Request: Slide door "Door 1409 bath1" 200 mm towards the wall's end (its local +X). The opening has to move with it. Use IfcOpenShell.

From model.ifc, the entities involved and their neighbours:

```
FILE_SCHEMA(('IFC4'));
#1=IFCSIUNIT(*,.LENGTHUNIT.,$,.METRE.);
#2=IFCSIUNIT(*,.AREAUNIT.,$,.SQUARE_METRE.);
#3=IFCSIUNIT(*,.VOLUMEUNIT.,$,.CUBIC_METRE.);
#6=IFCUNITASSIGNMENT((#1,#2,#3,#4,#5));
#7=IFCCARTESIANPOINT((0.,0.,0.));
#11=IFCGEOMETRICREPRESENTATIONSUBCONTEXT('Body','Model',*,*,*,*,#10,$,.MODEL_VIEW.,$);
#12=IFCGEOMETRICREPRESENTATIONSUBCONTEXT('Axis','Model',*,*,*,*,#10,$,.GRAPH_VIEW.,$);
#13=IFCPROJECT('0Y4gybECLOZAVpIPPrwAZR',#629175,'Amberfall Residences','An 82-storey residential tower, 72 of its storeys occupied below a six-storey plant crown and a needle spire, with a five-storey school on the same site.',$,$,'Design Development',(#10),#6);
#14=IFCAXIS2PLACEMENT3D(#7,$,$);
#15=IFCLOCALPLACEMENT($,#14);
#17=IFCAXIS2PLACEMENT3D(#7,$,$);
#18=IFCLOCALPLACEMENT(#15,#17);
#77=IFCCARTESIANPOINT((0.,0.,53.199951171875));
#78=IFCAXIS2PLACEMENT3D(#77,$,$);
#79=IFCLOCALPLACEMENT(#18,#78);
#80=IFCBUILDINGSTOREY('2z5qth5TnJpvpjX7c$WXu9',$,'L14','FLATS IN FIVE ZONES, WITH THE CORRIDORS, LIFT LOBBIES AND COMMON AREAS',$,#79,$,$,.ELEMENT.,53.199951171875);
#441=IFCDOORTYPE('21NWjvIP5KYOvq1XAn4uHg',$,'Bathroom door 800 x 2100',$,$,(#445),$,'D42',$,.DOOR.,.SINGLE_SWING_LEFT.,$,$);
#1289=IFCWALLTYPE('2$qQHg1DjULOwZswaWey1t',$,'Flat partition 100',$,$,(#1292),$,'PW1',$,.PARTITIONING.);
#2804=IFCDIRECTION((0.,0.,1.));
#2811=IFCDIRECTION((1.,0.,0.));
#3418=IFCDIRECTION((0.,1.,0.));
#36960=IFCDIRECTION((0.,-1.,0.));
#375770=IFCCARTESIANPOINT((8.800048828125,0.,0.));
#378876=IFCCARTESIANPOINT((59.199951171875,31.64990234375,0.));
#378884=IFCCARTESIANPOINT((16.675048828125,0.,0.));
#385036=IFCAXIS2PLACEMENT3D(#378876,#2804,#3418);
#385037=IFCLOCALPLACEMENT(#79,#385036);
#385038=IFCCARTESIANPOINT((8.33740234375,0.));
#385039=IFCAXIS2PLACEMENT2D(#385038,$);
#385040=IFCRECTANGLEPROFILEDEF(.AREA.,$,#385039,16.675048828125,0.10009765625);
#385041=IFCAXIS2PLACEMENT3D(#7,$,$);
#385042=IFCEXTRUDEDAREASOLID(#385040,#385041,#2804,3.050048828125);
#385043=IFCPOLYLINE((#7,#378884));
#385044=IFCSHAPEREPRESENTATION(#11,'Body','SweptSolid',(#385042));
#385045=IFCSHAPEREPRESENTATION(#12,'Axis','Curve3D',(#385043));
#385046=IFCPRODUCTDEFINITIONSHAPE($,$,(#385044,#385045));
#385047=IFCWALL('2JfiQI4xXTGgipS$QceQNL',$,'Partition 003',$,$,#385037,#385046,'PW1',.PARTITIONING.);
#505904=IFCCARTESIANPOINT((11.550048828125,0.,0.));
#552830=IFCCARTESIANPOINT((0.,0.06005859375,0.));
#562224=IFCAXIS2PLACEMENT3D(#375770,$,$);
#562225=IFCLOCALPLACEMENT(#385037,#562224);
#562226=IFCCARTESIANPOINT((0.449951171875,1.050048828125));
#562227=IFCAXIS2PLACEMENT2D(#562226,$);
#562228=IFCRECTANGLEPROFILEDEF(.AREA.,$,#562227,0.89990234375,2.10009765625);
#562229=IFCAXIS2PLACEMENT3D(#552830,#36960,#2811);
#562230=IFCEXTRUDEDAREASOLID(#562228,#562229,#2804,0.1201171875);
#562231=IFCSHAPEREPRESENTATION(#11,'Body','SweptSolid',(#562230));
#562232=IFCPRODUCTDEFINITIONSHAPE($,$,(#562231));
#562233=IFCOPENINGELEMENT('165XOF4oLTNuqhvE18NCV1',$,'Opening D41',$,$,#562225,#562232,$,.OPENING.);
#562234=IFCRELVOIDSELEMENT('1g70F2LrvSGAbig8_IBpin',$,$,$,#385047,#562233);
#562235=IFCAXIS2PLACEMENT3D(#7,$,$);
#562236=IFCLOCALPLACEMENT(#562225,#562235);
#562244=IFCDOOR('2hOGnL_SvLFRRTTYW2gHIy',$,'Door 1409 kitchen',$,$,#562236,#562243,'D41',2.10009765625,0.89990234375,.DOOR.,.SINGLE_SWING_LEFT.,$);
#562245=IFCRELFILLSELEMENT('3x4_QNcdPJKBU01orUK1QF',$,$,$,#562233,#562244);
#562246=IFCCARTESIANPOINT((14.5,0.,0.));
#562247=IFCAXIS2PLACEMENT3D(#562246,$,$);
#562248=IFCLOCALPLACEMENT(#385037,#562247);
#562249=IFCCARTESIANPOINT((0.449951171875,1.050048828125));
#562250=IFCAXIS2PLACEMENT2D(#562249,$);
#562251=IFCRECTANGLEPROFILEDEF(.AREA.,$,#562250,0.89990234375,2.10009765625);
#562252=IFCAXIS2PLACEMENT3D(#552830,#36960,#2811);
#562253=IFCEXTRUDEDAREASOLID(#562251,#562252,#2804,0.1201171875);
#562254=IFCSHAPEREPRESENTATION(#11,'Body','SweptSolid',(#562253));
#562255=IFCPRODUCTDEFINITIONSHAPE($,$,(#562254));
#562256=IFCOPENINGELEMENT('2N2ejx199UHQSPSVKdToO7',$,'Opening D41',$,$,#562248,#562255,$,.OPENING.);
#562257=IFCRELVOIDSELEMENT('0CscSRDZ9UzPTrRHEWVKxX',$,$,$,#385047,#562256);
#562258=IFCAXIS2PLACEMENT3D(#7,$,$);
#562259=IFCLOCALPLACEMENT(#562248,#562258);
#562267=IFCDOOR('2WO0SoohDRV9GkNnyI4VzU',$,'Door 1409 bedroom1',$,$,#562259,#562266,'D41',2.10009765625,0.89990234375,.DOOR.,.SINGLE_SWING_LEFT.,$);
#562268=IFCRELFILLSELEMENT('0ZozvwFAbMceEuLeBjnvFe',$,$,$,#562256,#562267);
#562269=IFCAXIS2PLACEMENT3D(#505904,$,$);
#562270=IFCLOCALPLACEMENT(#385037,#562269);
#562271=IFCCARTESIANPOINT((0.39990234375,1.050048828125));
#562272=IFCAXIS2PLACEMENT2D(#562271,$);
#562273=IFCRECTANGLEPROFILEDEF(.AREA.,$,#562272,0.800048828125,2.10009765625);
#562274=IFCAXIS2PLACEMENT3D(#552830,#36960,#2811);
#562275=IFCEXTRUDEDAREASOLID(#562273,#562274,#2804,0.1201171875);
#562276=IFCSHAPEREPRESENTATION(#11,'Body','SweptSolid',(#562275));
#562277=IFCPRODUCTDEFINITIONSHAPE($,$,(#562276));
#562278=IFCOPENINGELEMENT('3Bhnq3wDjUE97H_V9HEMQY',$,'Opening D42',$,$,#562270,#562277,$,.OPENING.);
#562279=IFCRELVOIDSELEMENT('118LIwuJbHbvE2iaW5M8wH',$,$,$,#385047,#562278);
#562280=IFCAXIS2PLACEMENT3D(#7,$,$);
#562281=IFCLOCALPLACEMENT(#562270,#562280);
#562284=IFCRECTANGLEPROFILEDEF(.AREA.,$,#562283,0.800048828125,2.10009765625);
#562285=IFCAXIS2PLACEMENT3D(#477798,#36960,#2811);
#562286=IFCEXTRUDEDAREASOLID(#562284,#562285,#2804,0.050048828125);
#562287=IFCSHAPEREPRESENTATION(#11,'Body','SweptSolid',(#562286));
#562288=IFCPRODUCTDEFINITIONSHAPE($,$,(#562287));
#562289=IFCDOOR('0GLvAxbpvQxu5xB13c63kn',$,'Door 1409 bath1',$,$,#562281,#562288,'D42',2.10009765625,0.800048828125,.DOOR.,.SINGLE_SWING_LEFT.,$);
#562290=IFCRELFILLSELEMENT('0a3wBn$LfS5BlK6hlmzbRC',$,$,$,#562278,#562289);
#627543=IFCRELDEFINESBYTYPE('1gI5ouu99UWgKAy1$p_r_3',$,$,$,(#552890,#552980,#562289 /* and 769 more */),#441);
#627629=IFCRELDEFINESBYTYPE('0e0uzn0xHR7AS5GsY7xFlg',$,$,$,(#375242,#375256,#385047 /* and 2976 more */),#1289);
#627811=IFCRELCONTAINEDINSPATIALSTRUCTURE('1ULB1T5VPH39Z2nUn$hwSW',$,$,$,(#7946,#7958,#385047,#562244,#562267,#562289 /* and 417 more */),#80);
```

```python
import ifcopenshell
import ifcopenshell.api.geometry
import ifcopenshell.util.placement

model = ifcopenshell.open("model.ifc")

door = model.by_id(562289)
opening = door.FillsVoids[0].RelatingOpeningElement
wall = opening.VoidsElements[0].RelatingBuildingElement

wall_matrix = ifcopenshell.util.placement.get_local_placement(wall.ObjectPlacement)
shift = wall_matrix[:3, 0] * 0.2
before = ifcopenshell.util.placement.get_local_placement(door.ObjectPlacement)[:3, 3].copy()

# The door is placed relative to its opening, so it follows when the opening moves.
matrix = ifcopenshell.util.placement.get_local_placement(opening.ObjectPlacement)
matrix[:3, 3] += shift
ifcopenshell.api.geometry.edit_object_placement(
    model, product=opening, matrix=matrix, is_si=False, should_transform_children=True
)

after = ifcopenshell.util.placement.get_local_placement(door.ObjectPlacement)[:3, 3]
print("door moved by", (after - before).round(3) + 0.0)

model.write("model_rev.ifc")
```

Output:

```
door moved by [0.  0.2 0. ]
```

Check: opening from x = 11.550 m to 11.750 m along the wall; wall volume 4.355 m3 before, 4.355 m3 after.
